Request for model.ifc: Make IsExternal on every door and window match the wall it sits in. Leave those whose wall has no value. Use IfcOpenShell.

First a look at what the model holds.

```python
import ifcopenshell
import ifcopenshell.util.element

model = ifcopenshell.open("model.ifc")
print(model.schema)
seen = {}
for e in model.by_type("IfcDoor") + model.by_type("IfcWindow"):
    if not e.FillsVoids:
        continue
    host = e.FillsVoids[0].RelatingOpeningElement.VoidsElements[0].RelatingBuildingElement
    own = ifcopenshell.util.element.get_pset(e, f"Pset_{e.is_a()[3:].removesuffix('StandardCase')}Common", "IsExternal")
    wall = ifcopenshell.util.element.get_pset(host, "Pset_WallCommon", "IsExternal")
    seen[e.is_a(), own, wall] = seen.get((e.is_a(), own, wall), 0) + 1
for (cls, own, wall), count in sorted(seen.items(), key=str):
    print(count, cls, "IsExternal:", own, "| host wall:", wall)
```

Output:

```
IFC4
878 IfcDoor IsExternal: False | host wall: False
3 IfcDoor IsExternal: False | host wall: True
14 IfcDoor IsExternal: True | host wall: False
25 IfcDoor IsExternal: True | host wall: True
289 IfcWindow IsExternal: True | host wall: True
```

```python
import ifcopenshell
import ifcopenshell.api.pset
import ifcopenshell.util.element

model = ifcopenshell.open("model.ifc")

count = 0
for ifc_class, pset_name in (("IfcDoor", "Pset_DoorCommon"), ("IfcWindow", "Pset_WindowCommon")):
    for e in model.by_type(ifc_class):
        if not e.FillsVoids:
            continue
        host = e.FillsVoids[0].RelatingOpeningElement.VoidsElements[0].RelatingBuildingElement
        external = ifcopenshell.util.element.get_pset(host, "Pset_WallCommon", "IsExternal")
        if external is None or ifcopenshell.util.element.get_pset(e, pset_name, "IsExternal") == external:
            continue
        pset = ifcopenshell.api.pset.add_pset(model, product=e, name=pset_name)
        ifcopenshell.api.pset.edit_pset(model, pset=pset, properties={"IsExternal": external})
        count += 1

print(count, "updated")

model.write("model-out.ifc")
```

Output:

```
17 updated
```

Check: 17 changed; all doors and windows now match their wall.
